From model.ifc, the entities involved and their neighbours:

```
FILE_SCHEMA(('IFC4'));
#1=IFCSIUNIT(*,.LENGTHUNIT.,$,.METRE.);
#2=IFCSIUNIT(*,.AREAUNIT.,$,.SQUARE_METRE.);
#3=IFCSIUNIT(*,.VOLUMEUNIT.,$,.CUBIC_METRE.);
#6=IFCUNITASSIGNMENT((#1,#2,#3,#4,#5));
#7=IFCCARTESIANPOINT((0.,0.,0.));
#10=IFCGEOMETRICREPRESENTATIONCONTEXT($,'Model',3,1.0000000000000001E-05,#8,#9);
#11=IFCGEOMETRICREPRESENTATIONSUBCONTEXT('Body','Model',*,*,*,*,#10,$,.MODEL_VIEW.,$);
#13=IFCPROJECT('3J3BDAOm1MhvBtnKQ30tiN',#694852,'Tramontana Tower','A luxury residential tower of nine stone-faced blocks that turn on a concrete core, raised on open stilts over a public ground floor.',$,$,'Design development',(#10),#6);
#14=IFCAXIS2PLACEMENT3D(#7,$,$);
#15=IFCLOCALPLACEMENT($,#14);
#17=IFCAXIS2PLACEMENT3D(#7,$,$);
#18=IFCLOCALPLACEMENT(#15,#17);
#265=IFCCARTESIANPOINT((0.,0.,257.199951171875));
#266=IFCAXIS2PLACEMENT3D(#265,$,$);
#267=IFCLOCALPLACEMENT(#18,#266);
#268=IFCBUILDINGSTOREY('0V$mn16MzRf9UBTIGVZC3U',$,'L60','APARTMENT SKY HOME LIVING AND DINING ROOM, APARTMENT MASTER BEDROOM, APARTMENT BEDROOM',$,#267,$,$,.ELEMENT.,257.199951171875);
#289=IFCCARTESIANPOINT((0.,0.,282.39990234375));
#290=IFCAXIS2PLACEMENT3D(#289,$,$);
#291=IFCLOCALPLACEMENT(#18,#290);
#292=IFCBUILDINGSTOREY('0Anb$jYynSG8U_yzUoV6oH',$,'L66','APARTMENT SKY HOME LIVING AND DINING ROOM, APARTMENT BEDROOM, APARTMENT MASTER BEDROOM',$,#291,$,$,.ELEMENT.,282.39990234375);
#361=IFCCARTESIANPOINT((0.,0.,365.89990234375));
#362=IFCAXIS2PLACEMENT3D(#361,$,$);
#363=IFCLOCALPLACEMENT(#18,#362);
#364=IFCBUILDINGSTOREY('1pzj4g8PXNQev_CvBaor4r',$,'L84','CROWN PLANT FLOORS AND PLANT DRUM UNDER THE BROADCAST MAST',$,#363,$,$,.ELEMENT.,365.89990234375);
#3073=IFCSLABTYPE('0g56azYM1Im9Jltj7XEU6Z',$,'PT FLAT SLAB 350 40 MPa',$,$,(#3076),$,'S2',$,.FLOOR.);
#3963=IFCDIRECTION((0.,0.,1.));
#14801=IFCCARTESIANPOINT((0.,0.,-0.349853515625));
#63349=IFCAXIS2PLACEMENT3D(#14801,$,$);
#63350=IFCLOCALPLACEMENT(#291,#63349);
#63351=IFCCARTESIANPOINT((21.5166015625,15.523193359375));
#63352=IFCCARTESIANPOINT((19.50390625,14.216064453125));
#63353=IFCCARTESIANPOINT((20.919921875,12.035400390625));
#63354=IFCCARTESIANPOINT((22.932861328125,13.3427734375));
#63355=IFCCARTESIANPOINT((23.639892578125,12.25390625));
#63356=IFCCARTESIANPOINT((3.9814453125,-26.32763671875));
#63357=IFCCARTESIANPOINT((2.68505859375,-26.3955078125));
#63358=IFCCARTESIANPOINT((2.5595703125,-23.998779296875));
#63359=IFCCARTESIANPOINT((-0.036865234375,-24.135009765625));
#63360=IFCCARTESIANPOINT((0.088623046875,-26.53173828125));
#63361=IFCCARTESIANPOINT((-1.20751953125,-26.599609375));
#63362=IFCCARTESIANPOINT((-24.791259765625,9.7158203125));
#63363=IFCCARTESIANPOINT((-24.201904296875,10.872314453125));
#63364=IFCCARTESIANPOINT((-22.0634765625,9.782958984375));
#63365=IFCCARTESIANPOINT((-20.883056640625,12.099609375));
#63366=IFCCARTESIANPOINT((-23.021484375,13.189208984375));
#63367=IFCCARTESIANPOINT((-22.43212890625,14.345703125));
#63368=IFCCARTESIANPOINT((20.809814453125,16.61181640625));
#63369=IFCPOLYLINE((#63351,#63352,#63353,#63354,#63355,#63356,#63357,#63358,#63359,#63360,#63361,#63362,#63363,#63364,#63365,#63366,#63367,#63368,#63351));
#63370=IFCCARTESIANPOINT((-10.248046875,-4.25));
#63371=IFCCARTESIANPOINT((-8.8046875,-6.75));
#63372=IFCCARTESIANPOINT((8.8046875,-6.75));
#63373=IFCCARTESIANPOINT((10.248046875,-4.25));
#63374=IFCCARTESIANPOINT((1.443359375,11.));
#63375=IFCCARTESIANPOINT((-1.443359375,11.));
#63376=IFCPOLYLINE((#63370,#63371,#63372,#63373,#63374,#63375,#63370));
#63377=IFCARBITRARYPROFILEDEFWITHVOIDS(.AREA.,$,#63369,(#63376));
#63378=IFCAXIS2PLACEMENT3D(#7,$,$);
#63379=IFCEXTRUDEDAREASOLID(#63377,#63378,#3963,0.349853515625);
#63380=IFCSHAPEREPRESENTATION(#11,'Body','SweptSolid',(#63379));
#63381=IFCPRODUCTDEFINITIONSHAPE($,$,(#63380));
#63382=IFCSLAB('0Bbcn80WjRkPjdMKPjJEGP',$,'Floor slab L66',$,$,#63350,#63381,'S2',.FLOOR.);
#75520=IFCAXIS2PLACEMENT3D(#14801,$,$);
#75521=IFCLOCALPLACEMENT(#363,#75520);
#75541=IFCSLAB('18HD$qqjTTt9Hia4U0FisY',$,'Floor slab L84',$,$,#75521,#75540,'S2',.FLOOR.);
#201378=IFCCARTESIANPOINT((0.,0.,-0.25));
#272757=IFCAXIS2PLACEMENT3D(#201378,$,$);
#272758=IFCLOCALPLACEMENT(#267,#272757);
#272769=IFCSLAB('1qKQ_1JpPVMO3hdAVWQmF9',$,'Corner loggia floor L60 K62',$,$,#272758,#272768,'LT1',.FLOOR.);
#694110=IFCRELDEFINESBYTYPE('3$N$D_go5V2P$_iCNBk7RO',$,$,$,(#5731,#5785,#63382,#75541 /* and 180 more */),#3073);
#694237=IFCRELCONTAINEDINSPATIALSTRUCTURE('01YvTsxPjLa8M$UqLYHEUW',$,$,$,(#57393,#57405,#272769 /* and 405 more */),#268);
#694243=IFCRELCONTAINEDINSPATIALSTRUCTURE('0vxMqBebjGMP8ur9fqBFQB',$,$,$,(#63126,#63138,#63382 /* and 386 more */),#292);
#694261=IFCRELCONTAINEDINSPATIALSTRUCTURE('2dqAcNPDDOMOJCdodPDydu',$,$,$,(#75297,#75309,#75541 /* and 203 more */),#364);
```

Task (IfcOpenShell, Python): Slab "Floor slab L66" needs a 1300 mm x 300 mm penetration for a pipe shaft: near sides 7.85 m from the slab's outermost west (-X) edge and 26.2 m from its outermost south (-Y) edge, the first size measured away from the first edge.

```python
import numpy as np
import ifcopenshell
import ifcopenshell.api.feature
import ifcopenshell.api.geometry
import ifcopenshell.api.root
import ifcopenshell.geom
import ifcopenshell.util.placement
import ifcopenshell.util.representation
import ifcopenshell.util.shape
import ifcopenshell.util.unit

model = ifcopenshell.open("model.ifc")
unit_scale = ifcopenshell.util.unit.calculate_unit_scale(model)
settings = ifcopenshell.geom.settings()


def volume(element):
    """Net volume in cubic metres, openings subtracted."""
    shape = ifcopenshell.geom.create_shape(settings, element)
    return ifcopenshell.util.shape.get_volume(shape.geometry)


slab = model.by_id(63382)
before = volume(slab)

# Extent in the slab's own axes, in metres. The edges named are its -X and -Y sides.
slab_shape = ifcopenshell.geom.create_shape(settings, slab)
vertices = ifcopenshell.util.shape.get_vertices(slab_shape.geometry)
x_min, y_min, bottom = vertices.min(axis=0)
top = vertices[:, 2].max()

opening = ifcopenshell.api.root.create_entity(model, ifc_class="IfcOpeningElement", name="Pipe shaft opening", predefined_type="OPENING")
context = ifcopenshell.util.representation.get_context(model, "Model", "Body", "MODEL_VIEW")
width, depth = 1.3, 0.3
outline = [(0.0, 0.0), (width, 0.0), (width, depth), (0.0, depth), (0.0, 0.0)]
# Overshoot both faces by 50 mm so the cut is clean.
shape = ifcopenshell.api.geometry.add_slab_representation(
    model, context=context, depth=top - bottom + 0.1, polyline=outline
)
ifcopenshell.api.geometry.assign_representation(model, product=opening, representation=shape)

matrix = ifcopenshell.util.placement.get_local_placement(slab.ObjectPlacement)
matrix[:, 3] = matrix @ np.append(np.array([x_min + 7.85, y_min + 26.2, bottom - 0.05]) / unit_scale, 1.0)
ifcopenshell.api.geometry.edit_object_placement(model, product=opening, matrix=matrix, is_si=False)
ifcopenshell.api.feature.add_feature(model, feature=opening, element=slab)

after = volume(slab)

print(f"slab volume {before:.3f} -> {after:.3f} m3")

model.write("model_updated.ifc")
```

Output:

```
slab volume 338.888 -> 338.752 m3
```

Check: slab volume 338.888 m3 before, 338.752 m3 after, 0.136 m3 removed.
